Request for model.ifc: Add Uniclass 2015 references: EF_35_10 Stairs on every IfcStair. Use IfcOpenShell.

First a look at what the model holds.

```python
import ifcopenshell

model = ifcopenshell.open("model.ifc")
print(model.schema)
print("classifications:", [c.Name for c in model.by_type("IfcClassification")])
for ifc_class in ("IfcDoor", "IfcRoof", "IfcStair", "IfcWall", "IfcWindow"):
    print(ifc_class, len(model.by_type(ifc_class)))
```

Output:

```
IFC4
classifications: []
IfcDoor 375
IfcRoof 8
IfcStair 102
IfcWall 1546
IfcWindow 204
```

```python
import ifcopenshell
import ifcopenshell.api.classification

model = ifcopenshell.open("model.ifc")

system = ifcopenshell.api.classification.add_classification(model, classification="Uniclass 2015")

codes = {
    "IfcStair": ("EF_35_10", "Stairs"),
}
for ifc_class, (code, name) in codes.items():
    products = model.by_type(ifc_class)
    ifcopenshell.api.classification.add_reference(
        model, products=products, classification=system, identification=code, name=name
    )
    print(code, len(products))

model.write("model-out.ifc")
```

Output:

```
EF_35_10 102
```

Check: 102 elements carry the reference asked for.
